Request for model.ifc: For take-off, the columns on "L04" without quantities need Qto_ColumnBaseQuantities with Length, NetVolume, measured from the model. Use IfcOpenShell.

First a look at what the model holds.

```python
import ifcopenshell
import ifcopenshell.util.element
import ifcopenshell.util.unit

model = ifcopenshell.open("model.ifc")
print(model.schema)
for unit_type in ("LENGTHUNIT", "AREAUNIT", "VOLUMEUNIT"):
    print(unit_type, ifcopenshell.util.unit.calculate_unit_scale(model, unit_type))
storey = next(s for s in model.by_type("IfcBuildingStorey") if s.Name == "L04")
columns = [e for e in ifcopenshell.util.element.get_decomposition(storey) if e.is_a("IfcColumn")]
for e in sorted(columns, key=lambda e: e.id()):
    print(e.id(), e.is_a(), e.Name, list(ifcopenshell.util.element.get_psets(e, qtos_only=True)), sep=" | ")
```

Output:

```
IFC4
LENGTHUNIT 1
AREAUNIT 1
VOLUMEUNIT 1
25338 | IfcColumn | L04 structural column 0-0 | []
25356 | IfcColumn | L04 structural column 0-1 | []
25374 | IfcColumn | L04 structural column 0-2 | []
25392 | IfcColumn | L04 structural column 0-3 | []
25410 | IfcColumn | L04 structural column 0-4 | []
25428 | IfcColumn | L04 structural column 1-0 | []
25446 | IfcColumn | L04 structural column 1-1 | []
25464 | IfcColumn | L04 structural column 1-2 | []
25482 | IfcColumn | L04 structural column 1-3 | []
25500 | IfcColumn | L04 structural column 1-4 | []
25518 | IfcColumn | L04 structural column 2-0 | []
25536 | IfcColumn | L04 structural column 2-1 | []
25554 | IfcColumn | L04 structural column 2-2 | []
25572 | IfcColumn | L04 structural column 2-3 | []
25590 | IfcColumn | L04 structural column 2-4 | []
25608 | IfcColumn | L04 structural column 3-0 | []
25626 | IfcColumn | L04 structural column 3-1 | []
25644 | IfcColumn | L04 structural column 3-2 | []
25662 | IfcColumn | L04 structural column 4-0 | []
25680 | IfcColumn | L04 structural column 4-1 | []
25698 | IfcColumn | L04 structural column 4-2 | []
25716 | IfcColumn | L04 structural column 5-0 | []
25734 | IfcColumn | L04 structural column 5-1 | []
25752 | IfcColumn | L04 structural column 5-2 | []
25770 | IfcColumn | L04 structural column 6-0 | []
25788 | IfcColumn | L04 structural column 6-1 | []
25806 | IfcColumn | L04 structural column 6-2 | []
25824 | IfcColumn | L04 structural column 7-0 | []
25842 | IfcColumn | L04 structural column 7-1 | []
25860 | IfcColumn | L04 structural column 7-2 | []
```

```python
import ifcopenshell
import ifcopenshell.api.pset
import ifcopenshell.geom
import ifcopenshell.util.element
import ifcopenshell.util.shape
import ifcopenshell.util.unit

model = ifcopenshell.open("model.ifc")
unit_scale = ifcopenshell.util.unit.calculate_unit_scale(model)
volume_scale = ifcopenshell.util.unit.calculate_unit_scale(model, "VOLUMEUNIT")
settings = ifcopenshell.geom.settings()

storey = next(s for s in model.by_type("IfcBuildingStorey") if s.Name == "L04")
columns = [e for e in ifcopenshell.util.element.get_decomposition(storey) if e.is_a("IfcColumn")]

for e in sorted(columns, key=lambda e: e.id()):
    if ifcopenshell.util.element.get_psets(e, qtos_only=True, should_inherit=False):
        continue
    # Geometry comes back in metres, in the element's own axes.
    shape = ifcopenshell.geom.create_shape(settings, e)
    values = {
        "Length": ifcopenshell.util.shape.get_z(shape.geometry) / unit_scale,
        "NetVolume": ifcopenshell.util.shape.get_volume(shape.geometry) / volume_scale,
    }
    qto = ifcopenshell.api.pset.add_qto(model, product=e, name="Qto_ColumnBaseQuantities")
    ifcopenshell.api.pset.edit_qto(model, qto=qto, properties=values)
    print(e.id(), {k: round(v, 3) for k, v in values.items()})

model.write("model_rev.ifc")
```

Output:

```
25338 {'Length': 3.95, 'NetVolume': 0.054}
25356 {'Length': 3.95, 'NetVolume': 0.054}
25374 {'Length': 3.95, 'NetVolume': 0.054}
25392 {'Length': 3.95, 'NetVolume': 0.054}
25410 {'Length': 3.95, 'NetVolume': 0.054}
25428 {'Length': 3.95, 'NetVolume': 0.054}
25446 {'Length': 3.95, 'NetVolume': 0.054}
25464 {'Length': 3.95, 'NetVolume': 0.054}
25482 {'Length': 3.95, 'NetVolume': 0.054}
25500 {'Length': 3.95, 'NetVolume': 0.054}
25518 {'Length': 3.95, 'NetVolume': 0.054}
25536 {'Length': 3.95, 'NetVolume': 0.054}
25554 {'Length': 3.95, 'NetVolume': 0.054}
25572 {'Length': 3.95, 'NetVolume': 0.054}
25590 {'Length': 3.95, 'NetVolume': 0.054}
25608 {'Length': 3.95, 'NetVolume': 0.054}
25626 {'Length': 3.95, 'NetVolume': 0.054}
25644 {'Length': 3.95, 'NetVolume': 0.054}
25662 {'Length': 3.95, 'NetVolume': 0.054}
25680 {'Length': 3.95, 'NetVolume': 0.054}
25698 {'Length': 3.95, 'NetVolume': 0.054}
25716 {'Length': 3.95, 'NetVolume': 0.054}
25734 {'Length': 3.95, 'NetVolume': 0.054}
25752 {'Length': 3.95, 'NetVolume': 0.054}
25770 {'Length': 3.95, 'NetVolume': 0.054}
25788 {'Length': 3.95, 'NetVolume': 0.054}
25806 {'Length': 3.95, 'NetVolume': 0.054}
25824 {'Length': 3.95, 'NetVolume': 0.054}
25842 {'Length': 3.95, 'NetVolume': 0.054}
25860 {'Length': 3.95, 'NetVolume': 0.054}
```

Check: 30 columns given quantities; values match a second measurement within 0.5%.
